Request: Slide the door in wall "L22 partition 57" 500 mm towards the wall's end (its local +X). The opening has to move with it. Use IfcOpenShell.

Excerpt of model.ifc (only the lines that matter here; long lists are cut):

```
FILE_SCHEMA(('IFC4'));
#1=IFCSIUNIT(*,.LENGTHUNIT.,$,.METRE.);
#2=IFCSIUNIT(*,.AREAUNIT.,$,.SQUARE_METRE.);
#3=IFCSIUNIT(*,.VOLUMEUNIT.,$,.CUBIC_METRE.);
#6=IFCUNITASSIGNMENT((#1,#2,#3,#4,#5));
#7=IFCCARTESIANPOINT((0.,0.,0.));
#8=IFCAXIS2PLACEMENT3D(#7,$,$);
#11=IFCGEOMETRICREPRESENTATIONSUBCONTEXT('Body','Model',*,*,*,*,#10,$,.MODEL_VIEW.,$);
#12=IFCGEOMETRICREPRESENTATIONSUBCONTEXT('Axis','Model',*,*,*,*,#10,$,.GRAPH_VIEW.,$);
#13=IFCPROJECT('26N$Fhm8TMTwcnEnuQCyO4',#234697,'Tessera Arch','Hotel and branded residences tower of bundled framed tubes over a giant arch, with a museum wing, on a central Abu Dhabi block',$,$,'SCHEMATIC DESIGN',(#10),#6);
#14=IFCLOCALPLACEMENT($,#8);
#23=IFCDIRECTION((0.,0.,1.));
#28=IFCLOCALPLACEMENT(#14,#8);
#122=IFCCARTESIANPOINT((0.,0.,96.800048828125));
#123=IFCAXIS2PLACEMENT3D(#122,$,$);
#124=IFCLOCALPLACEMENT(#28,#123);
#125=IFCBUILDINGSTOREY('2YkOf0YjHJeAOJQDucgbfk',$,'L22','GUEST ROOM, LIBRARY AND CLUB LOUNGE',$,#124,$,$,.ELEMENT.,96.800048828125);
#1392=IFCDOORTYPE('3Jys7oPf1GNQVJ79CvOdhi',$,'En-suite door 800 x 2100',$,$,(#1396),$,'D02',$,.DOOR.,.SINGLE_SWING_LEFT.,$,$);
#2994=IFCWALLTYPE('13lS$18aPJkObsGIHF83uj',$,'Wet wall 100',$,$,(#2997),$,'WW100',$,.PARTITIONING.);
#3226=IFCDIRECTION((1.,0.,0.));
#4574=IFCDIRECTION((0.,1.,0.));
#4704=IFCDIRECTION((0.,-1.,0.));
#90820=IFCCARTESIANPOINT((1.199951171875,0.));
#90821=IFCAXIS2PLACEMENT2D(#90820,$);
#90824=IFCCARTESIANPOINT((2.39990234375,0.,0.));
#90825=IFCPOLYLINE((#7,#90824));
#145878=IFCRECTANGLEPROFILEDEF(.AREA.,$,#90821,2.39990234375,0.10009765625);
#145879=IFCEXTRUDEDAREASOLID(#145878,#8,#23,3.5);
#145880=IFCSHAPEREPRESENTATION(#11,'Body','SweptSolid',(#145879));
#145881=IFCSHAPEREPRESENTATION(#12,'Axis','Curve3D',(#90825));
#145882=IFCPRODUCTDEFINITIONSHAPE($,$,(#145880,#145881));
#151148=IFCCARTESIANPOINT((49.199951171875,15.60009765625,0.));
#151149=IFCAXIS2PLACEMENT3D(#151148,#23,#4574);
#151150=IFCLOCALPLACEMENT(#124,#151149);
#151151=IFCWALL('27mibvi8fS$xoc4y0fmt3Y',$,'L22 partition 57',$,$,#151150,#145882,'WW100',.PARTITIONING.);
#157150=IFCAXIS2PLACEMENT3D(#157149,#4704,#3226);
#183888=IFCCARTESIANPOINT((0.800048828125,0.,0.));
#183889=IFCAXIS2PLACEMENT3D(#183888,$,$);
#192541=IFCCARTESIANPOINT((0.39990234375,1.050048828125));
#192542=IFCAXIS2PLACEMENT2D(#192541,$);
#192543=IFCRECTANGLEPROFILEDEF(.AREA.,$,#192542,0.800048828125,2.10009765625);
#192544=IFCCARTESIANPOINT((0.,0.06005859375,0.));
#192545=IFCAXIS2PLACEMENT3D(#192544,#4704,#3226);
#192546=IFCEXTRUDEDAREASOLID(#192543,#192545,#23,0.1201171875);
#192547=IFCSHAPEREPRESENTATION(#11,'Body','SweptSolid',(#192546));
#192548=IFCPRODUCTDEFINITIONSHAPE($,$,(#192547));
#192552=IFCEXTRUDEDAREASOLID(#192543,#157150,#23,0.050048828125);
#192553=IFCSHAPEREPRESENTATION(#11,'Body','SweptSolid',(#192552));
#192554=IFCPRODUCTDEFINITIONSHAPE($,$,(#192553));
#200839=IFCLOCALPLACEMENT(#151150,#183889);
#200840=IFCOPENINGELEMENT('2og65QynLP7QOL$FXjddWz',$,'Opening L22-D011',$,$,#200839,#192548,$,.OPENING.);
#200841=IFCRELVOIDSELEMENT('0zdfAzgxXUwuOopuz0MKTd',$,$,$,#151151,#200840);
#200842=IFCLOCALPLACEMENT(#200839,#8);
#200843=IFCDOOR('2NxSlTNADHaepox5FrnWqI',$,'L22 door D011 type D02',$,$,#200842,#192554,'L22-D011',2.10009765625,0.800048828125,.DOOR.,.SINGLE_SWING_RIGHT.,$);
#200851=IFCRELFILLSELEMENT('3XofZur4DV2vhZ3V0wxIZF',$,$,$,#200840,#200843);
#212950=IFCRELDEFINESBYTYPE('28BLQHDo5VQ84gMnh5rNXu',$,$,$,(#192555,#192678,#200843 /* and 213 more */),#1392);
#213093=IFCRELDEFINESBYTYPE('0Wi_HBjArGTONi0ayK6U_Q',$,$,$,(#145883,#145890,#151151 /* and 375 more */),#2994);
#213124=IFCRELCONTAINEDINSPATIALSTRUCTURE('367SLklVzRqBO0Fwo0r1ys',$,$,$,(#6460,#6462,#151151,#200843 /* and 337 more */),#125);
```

```python
import ifcopenshell
import ifcopenshell.api.geometry
import ifcopenshell.util.placement
import ifcopenshell.util.unit

model = ifcopenshell.open("model.ifc")
unit_scale = ifcopenshell.util.unit.calculate_unit_scale(model)

door = model.by_id(200843)
opening = door.FillsVoids[0].RelatingOpeningElement
wall = opening.VoidsElements[0].RelatingBuildingElement

wall_matrix = ifcopenshell.util.placement.get_local_placement(wall.ObjectPlacement)
shift = wall_matrix[:3, 0] * 0.5 / unit_scale
before = ifcopenshell.util.placement.get_local_placement(door.ObjectPlacement)[:3, 3].copy()

# The door is placed relative to its opening, so it follows when the opening moves.
matrix = ifcopenshell.util.placement.get_local_placement(opening.ObjectPlacement)
matrix[:3, 3] += shift
ifcopenshell.api.geometry.edit_object_placement(
    model, product=opening, matrix=matrix, is_si=False, should_transform_children=True
)

after = ifcopenshell.util.placement.get_local_placement(door.ObjectPlacement)[:3, 3]
print("door moved by", (after - before).round(3) + 0.0)

model.write("model_v2.ifc")
```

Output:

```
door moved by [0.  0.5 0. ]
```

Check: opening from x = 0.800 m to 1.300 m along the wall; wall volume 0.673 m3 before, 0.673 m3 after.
